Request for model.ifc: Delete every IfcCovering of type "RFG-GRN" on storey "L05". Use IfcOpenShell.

First a look at what the model holds.

```python
import ifcopenshell
import ifcopenshell.util.element

model = ifcopenshell.open("model.ifc")
print(model.schema)
storey = next(s for s in model.by_type("IfcBuildingStorey") if s.Name == "L05")
coverings = [e for e in ifcopenshell.util.element.get_decomposition(storey) if e.is_a("IfcCovering")]
seen = {}
for e in coverings:
    element_type = ifcopenshell.util.element.get_type(e)
    name = element_type.Name if element_type not in (None, e) else None
    seen[name] = seen.get(name, 0) + 1
for name, count in sorted(seen.items(), key=str):
    print(count, "x", name)
```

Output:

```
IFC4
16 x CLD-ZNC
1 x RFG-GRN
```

```python
import ifcopenshell
import ifcopenshell.api.root
import ifcopenshell.util.element

model = ifcopenshell.open("model.ifc")

storey = next(s for s in model.by_type("IfcBuildingStorey") if s.Name == "L05")
coverings = [e for e in ifcopenshell.util.element.get_decomposition(storey) if e.is_a("IfcCovering")]
targets = [e for e in coverings if (t := ifcopenshell.util.element.get_type(e)) not in (None, e) and t.Name == "RFG-GRN"]

for e in targets:
    ifcopenshell.api.root.remove_product(model, product=e)
print(len(targets), "removed")

model.write("model-out.ifc")
```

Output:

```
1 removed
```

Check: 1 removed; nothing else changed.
